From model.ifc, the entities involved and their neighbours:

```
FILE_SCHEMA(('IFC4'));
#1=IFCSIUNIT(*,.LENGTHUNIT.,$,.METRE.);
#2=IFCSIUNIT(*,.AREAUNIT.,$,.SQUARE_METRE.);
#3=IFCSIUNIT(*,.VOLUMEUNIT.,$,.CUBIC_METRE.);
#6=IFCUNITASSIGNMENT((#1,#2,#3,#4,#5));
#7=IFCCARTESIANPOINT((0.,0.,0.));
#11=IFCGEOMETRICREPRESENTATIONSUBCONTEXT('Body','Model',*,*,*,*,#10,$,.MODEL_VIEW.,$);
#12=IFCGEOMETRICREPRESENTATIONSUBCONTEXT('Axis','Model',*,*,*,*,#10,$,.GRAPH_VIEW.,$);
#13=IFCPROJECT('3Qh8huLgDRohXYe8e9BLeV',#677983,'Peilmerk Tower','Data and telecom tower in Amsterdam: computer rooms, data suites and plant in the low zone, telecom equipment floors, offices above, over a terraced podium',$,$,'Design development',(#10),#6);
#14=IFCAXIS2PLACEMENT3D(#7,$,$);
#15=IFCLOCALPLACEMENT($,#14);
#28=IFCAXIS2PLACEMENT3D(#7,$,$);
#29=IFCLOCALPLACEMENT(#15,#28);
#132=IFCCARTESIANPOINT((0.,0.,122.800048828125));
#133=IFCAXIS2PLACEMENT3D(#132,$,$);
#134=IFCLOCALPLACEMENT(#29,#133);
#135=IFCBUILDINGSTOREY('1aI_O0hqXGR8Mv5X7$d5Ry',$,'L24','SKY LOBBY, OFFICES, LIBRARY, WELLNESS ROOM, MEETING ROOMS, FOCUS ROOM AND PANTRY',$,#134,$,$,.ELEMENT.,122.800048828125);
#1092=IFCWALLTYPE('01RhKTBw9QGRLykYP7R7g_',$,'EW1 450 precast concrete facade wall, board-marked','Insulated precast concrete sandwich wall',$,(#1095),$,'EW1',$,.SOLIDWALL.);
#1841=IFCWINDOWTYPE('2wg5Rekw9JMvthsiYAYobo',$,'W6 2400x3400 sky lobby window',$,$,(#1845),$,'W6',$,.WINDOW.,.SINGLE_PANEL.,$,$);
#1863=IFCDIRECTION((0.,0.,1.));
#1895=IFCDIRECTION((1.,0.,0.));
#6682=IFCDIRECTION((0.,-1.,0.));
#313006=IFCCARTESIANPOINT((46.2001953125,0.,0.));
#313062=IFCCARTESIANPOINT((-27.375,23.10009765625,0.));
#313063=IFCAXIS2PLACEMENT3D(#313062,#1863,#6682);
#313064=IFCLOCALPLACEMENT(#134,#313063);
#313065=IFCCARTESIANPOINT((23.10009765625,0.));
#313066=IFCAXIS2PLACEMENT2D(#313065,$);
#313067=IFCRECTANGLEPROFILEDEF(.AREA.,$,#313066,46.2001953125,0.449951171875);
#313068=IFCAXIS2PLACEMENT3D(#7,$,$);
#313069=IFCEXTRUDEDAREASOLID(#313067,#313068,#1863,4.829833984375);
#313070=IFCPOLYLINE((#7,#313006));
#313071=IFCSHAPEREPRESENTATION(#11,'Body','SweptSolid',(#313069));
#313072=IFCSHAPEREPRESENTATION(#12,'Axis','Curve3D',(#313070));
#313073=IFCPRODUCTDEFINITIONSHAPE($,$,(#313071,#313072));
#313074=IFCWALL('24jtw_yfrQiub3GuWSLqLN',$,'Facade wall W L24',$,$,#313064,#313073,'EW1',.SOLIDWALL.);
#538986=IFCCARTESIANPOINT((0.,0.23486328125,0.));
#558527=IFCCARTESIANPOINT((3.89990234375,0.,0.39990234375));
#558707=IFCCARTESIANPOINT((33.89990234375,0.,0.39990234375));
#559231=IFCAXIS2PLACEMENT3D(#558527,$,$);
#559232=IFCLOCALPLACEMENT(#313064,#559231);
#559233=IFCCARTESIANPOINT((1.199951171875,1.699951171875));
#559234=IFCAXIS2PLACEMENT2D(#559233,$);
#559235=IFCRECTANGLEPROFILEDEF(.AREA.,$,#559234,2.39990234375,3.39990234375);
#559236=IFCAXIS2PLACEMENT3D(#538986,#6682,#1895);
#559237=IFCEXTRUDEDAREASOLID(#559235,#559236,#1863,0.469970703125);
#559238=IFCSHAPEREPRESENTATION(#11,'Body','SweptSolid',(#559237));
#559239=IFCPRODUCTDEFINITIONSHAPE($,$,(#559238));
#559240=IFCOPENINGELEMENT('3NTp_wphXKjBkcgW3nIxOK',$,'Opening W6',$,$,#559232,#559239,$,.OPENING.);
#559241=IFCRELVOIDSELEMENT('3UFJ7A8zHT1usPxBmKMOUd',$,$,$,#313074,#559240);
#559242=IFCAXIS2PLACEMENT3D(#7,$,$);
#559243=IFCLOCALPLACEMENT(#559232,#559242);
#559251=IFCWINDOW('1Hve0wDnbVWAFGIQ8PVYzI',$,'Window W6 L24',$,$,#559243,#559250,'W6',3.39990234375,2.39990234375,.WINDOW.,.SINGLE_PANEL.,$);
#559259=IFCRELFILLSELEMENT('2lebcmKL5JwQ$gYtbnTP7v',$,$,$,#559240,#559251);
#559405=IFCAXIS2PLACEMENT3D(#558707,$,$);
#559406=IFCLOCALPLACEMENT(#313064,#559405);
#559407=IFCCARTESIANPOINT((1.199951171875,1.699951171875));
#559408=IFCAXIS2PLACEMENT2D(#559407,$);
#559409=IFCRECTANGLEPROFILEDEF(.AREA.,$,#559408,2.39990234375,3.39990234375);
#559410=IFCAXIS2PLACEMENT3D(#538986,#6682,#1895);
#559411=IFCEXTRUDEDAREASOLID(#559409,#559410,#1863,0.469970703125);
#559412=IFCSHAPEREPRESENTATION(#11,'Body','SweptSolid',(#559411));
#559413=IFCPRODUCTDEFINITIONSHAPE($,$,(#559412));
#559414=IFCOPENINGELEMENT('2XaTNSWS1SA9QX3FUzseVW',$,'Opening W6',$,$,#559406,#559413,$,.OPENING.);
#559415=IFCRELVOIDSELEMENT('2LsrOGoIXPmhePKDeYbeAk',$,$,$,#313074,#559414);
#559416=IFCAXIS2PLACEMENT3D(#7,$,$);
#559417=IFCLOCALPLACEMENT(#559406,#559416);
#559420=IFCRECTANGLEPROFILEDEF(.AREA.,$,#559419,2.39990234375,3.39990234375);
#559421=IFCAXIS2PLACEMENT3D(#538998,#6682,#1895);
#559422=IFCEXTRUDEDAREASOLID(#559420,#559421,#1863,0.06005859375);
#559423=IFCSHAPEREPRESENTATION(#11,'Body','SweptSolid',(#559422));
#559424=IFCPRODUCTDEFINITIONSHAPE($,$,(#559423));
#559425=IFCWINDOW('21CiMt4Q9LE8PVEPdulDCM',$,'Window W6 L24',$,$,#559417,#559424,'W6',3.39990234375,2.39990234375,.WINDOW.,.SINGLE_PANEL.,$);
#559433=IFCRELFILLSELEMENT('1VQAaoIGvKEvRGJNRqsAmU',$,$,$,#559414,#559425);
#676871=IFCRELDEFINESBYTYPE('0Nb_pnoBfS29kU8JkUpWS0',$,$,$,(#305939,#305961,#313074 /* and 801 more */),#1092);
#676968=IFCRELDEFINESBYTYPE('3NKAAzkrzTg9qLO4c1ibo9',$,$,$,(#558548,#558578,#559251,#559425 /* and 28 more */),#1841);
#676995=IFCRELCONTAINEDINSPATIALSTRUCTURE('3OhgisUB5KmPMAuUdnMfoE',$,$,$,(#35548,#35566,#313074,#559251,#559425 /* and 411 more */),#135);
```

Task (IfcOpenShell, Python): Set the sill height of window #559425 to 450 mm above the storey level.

```python
import numpy as np
import ifcopenshell
import ifcopenshell.api.geometry
import ifcopenshell.geom
import ifcopenshell.util.element
import ifcopenshell.util.placement
import ifcopenshell.util.shape
import ifcopenshell.util.unit

model = ifcopenshell.open("model.ifc")
unit_scale = ifcopenshell.util.unit.calculate_unit_scale(model)

window = model.by_guid("21CiMt4Q9LE8PVEPdulDCM")
opening = window.FillsVoids[0].RelatingOpeningElement
storey = ifcopenshell.util.element.get_container(window, ifc_class="IfcBuildingStorey")
level = ifcopenshell.util.placement.get_local_placement(storey.ObjectPlacement)[2, 3]

# The opening's origin need not be at the sill, so measure its lowest point.
shape = ifcopenshell.geom.create_shape(ifcopenshell.geom.settings(), opening)
bottom = ifcopenshell.util.shape.get_shape_bottom_elevation(shape, shape.geometry) / unit_scale
dz = level + 0.45 / unit_scale - bottom

shift = np.array([0.0, 0.0, dz])
# The window is placed relative to its opening, so it follows when the opening moves.
matrix = ifcopenshell.util.placement.get_local_placement(opening.ObjectPlacement)
matrix[:3, 3] += shift
ifcopenshell.api.geometry.edit_object_placement(
    model, product=opening, matrix=matrix, is_si=False, should_transform_children=True
)

print(f"moved by {dz * unit_scale:+.3f} m")

model.write("model_v2.ifc")
```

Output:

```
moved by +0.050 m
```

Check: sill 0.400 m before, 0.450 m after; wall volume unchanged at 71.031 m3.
